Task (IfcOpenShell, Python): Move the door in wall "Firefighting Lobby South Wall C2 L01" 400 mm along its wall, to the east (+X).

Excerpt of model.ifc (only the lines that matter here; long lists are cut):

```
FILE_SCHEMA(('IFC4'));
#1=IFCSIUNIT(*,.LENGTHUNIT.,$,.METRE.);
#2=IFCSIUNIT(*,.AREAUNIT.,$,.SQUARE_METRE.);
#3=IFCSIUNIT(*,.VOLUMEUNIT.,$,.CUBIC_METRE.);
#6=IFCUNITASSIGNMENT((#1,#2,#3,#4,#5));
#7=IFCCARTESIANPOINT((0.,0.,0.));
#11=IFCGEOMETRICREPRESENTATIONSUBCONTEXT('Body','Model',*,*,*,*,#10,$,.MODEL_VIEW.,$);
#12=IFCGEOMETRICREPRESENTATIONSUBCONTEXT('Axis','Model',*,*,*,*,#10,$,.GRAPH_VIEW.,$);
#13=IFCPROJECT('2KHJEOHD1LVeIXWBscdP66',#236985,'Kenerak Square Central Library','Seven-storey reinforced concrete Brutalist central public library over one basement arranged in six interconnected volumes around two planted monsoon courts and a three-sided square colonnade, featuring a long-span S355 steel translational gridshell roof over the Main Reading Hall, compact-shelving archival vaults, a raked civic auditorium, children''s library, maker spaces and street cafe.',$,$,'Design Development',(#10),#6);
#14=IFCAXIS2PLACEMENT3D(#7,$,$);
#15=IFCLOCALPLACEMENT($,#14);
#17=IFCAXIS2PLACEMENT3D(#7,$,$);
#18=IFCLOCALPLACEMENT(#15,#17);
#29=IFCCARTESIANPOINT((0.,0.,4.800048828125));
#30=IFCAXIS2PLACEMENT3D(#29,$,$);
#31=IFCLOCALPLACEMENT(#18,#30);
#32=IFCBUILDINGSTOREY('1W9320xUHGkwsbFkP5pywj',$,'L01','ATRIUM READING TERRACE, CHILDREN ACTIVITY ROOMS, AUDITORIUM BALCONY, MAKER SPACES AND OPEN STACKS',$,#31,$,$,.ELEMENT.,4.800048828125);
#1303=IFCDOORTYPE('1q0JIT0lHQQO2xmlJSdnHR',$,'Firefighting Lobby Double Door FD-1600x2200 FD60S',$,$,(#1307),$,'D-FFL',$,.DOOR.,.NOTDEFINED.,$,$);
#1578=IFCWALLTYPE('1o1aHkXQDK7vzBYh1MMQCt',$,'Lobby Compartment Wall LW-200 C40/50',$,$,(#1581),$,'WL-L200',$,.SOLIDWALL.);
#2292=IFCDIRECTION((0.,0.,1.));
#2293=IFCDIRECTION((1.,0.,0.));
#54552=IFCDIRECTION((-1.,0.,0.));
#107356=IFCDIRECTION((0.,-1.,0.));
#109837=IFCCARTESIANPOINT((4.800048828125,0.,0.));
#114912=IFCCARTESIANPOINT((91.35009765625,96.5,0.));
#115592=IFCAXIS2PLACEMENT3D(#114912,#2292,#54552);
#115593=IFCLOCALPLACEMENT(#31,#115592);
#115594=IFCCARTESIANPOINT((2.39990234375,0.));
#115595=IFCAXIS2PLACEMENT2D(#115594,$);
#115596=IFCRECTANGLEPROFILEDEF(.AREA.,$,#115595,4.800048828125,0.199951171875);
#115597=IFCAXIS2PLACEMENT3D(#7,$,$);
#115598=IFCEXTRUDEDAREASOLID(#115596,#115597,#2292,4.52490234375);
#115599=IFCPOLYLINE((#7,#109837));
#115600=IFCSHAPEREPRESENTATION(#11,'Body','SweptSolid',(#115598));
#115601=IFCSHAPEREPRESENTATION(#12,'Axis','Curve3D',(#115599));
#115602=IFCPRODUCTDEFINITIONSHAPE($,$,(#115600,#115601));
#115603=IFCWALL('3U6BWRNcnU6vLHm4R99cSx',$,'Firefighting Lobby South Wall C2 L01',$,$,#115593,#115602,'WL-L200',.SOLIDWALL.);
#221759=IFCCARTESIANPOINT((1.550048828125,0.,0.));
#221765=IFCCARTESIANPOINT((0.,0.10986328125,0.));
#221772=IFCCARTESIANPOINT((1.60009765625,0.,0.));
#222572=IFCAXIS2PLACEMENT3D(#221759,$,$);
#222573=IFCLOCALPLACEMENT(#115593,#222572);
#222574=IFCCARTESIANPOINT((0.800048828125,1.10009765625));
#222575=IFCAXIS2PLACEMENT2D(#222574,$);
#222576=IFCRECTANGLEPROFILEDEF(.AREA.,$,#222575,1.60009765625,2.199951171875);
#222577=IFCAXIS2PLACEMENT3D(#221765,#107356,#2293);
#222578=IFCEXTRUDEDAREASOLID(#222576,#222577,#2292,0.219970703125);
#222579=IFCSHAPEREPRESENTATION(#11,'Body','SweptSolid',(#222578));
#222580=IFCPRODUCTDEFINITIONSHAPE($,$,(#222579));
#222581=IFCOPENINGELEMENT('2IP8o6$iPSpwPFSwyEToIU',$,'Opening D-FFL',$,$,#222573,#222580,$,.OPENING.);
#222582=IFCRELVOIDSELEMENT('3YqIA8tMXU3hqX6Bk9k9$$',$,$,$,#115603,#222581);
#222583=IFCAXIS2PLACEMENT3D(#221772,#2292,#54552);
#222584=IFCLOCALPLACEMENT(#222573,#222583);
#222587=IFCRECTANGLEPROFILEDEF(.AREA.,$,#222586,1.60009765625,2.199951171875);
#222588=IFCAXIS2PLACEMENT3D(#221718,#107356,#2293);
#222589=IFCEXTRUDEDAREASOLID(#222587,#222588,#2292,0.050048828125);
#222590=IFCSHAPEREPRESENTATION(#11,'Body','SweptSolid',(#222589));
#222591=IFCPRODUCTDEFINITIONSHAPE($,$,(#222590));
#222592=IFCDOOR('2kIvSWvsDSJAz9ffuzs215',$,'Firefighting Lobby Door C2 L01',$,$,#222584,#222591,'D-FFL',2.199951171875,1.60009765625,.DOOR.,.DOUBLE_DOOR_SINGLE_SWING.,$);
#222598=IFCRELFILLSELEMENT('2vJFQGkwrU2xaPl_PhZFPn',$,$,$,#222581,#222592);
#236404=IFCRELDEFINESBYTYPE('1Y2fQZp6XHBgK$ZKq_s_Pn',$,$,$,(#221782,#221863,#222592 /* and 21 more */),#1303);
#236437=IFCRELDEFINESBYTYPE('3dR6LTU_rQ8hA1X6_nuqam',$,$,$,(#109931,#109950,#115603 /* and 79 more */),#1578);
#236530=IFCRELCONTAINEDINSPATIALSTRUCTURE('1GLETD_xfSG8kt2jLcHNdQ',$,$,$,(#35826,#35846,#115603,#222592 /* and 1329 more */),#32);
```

```python
import ifcopenshell
import ifcopenshell.api.geometry
import ifcopenshell.util.placement

model = ifcopenshell.open("model.ifc")

door = model.by_guid("2kIvSWvsDSJAz9ffuzs215")
opening = door.FillsVoids[0].RelatingOpeningElement
wall = opening.VoidsElements[0].RelatingBuildingElement

wall_matrix = ifcopenshell.util.placement.get_local_placement(wall.ObjectPlacement)
shift = wall_matrix[:3, 0] * -0.4
before = ifcopenshell.util.placement.get_local_placement(door.ObjectPlacement)[:3, 3].copy()

# The door is placed relative to its opening, so it follows when the opening moves.
matrix = ifcopenshell.util.placement.get_local_placement(opening.ObjectPlacement)
matrix[:3, 3] += shift
ifcopenshell.api.geometry.edit_object_placement(
    model, product=opening, matrix=matrix, is_si=False, should_transform_children=True
)

after = ifcopenshell.util.placement.get_local_placement(door.ObjectPlacement)[:3, 3]
print("door moved by", (after - before).round(3) + 0.0)

model.write("model_v2.ifc")
```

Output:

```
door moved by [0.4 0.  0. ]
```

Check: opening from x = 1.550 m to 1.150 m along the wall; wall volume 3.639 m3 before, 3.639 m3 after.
